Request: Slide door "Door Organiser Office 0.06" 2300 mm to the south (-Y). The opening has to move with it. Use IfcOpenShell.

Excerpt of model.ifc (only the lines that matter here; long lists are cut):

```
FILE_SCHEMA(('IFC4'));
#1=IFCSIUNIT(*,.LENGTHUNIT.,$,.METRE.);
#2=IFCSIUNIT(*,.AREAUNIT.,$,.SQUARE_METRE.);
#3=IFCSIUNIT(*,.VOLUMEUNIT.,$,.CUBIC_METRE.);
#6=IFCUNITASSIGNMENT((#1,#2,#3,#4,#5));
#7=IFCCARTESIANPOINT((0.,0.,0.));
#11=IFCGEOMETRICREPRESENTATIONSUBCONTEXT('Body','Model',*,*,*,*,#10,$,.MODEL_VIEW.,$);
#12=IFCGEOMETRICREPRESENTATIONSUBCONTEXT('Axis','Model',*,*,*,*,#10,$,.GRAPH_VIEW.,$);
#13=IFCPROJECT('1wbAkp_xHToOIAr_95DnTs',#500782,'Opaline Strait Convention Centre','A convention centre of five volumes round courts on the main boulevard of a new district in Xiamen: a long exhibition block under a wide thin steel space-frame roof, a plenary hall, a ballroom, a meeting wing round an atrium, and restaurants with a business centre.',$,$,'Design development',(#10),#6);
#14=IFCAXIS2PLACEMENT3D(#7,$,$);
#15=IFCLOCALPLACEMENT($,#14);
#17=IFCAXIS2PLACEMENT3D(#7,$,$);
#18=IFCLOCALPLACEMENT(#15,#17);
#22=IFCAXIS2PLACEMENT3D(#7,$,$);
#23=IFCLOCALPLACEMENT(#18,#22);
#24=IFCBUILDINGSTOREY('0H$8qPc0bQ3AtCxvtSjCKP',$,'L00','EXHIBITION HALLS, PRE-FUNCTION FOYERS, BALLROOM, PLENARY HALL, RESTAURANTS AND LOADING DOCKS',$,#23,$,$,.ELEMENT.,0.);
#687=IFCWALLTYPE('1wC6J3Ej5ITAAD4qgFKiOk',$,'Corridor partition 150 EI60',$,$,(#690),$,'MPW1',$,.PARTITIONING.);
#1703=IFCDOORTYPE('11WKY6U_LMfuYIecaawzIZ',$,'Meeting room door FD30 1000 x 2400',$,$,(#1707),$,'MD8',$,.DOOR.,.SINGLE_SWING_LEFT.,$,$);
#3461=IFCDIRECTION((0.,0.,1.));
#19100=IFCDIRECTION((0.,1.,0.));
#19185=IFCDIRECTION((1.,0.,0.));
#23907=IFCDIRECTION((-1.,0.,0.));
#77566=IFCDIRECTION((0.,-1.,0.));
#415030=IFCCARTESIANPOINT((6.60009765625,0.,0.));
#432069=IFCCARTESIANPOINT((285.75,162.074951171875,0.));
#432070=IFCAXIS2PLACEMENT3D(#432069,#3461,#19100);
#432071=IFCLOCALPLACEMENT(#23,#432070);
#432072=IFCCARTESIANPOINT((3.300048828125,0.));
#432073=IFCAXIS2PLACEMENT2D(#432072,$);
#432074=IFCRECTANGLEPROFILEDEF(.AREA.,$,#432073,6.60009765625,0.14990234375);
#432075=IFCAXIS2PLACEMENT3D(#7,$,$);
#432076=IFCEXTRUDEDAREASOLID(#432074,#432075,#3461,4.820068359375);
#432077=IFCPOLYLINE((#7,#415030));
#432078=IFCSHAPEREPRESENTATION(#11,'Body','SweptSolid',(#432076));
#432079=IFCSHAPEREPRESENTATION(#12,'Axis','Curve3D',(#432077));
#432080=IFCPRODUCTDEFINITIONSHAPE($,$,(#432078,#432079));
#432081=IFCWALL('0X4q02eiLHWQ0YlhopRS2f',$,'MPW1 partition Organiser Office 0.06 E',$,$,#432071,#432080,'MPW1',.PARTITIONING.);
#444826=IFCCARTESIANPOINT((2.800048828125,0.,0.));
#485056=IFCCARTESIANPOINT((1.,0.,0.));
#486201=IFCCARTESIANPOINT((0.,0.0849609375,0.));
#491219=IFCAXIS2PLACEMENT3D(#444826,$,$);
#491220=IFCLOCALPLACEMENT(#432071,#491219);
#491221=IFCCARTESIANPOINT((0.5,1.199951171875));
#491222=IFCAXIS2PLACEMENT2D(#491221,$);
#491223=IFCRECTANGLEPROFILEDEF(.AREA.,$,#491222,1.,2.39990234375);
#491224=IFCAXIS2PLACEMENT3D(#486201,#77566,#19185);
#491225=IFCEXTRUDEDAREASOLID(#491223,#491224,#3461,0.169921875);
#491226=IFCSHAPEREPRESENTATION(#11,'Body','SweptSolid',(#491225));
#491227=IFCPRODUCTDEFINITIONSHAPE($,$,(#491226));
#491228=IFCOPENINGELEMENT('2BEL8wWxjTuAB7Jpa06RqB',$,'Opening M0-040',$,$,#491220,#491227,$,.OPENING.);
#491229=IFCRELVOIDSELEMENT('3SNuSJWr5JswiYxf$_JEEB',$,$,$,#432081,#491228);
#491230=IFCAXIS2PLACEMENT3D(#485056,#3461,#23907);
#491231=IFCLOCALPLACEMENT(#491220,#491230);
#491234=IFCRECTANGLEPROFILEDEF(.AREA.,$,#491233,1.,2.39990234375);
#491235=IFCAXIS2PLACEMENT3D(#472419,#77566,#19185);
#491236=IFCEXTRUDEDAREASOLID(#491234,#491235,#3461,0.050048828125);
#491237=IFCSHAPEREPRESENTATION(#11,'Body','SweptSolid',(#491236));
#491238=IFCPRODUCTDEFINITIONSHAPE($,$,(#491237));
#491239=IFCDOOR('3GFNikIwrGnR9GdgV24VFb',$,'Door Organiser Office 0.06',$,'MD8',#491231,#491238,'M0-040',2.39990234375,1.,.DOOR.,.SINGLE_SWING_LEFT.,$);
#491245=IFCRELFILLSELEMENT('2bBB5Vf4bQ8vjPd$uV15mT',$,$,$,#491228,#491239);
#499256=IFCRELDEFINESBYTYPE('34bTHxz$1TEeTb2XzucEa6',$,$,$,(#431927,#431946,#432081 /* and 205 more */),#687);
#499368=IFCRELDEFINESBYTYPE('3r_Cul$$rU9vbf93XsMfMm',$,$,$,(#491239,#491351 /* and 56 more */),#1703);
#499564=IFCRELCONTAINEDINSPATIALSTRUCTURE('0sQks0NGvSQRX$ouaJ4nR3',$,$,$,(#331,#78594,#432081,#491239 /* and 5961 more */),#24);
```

```python
import ifcopenshell
import ifcopenshell.api.geometry
import ifcopenshell.util.placement
import ifcopenshell.util.unit

model = ifcopenshell.open("model.ifc")
unit_scale = ifcopenshell.util.unit.calculate_unit_scale(model)

door = model.by_id(491239)
opening = door.FillsVoids[0].RelatingOpeningElement
wall = opening.VoidsElements[0].RelatingBuildingElement

wall_matrix = ifcopenshell.util.placement.get_local_placement(wall.ObjectPlacement)
shift = wall_matrix[:3, 0] * -2.3 / unit_scale
before = ifcopenshell.util.placement.get_local_placement(door.ObjectPlacement)[:3, 3].copy()

# The door is placed relative to its opening, so it follows when the opening moves.
matrix = ifcopenshell.util.placement.get_local_placement(opening.ObjectPlacement)
matrix[:3, 3] += shift
ifcopenshell.api.geometry.edit_object_placement(
    model, product=opening, matrix=matrix, is_si=False, should_transform_children=True
)

after = ifcopenshell.util.placement.get_local_placement(door.ObjectPlacement)[:3, 3]
print("door moved by", (after - before).round(3) + 0.0)

model.write("model_v2.ifc")
```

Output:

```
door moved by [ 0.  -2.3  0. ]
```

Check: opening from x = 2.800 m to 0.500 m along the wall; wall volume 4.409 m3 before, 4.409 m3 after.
